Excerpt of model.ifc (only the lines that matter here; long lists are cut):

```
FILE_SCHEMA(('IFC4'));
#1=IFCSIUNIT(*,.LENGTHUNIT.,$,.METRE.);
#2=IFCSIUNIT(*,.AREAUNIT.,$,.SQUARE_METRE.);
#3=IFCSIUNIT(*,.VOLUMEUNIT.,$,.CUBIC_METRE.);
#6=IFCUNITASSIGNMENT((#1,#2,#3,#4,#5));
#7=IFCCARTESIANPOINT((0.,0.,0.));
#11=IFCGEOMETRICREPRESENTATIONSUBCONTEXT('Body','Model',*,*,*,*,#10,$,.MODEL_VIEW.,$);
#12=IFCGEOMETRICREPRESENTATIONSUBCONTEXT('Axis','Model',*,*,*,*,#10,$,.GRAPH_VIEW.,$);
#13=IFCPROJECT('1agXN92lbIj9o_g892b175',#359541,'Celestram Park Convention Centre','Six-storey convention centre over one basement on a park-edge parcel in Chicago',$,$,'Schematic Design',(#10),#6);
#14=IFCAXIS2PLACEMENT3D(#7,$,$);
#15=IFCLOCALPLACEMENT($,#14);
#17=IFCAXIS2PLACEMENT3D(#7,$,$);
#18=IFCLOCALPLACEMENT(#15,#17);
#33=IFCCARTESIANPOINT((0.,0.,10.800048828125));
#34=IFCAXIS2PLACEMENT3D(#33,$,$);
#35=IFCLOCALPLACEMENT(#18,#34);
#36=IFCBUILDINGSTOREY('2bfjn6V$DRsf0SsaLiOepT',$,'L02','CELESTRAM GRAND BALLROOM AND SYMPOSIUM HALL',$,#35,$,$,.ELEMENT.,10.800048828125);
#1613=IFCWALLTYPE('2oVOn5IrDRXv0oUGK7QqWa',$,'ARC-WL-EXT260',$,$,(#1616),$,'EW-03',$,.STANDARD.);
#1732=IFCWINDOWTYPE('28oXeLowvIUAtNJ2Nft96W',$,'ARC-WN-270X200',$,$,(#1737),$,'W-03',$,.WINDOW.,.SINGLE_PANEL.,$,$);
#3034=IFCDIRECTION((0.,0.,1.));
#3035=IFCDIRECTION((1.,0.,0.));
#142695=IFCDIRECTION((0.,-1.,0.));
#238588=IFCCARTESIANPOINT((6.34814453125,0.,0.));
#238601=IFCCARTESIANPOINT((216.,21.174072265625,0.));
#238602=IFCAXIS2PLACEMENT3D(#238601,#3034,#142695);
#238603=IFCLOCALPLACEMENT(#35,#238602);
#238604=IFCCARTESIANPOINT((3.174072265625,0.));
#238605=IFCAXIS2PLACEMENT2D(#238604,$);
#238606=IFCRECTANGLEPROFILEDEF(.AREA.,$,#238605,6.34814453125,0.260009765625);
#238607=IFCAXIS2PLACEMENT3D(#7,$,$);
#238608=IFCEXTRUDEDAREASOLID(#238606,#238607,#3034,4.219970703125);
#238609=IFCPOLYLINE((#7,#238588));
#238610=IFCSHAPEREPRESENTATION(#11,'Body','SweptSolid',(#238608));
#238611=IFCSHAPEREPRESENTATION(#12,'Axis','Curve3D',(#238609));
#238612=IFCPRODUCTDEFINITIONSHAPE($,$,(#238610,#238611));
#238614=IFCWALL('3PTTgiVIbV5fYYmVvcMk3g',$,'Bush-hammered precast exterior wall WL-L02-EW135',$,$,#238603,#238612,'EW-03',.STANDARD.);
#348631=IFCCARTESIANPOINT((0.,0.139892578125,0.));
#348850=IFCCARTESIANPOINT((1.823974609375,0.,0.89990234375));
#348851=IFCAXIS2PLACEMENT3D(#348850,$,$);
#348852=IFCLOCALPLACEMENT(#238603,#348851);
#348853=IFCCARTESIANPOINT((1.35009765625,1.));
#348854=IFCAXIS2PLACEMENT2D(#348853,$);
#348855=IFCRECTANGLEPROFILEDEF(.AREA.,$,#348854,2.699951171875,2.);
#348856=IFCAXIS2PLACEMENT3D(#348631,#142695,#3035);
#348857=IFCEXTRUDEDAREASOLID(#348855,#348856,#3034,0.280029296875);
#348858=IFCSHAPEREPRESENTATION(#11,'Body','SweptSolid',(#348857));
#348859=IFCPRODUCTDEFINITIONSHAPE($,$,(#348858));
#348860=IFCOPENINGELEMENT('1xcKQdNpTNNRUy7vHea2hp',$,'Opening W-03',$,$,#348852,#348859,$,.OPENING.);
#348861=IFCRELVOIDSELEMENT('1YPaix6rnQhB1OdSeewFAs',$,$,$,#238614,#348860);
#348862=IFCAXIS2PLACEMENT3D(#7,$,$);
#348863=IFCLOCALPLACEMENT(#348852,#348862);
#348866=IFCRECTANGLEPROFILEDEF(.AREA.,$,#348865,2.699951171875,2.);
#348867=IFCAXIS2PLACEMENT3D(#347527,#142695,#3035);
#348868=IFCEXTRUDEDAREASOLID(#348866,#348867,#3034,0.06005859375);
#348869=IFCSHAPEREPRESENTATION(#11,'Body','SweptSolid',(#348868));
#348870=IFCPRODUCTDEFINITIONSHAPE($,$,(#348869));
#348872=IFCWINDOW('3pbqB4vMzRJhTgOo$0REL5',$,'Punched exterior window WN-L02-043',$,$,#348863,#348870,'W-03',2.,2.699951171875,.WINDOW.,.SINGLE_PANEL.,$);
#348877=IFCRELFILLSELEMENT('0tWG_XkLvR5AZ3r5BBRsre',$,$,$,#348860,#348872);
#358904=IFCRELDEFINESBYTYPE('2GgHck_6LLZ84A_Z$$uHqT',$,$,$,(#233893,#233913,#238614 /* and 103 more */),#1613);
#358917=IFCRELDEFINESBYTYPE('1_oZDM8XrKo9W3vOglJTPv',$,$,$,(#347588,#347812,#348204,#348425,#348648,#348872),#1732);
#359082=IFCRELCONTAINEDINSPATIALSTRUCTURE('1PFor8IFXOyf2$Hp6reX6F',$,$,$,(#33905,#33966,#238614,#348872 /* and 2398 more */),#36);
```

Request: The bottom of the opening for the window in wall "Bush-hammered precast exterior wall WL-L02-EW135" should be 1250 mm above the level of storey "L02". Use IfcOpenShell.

```python
import numpy as np
import ifcopenshell
import ifcopenshell.api.geometry
import ifcopenshell.geom
import ifcopenshell.util.element
import ifcopenshell.util.placement
import ifcopenshell.util.shape
import ifcopenshell.util.unit

model = ifcopenshell.open("model.ifc")
unit_scale = ifcopenshell.util.unit.calculate_unit_scale(model)

window = model.by_id(348872)
opening = window.FillsVoids[0].RelatingOpeningElement
storey = ifcopenshell.util.element.get_container(window, ifc_class="IfcBuildingStorey")
level = ifcopenshell.util.placement.get_local_placement(storey.ObjectPlacement)[2, 3]

# The opening's origin need not be at the sill, so measure its lowest point.
shape = ifcopenshell.geom.create_shape(ifcopenshell.geom.settings(), opening)
bottom = ifcopenshell.util.shape.get_shape_bottom_elevation(shape, shape.geometry) / unit_scale
dz = level + 1.25 - bottom

shift = np.array([0.0, 0.0, dz])
# The window is placed relative to its opening, so it follows when the opening moves.
matrix = ifcopenshell.util.placement.get_local_placement(opening.ObjectPlacement)
matrix[:3, 3] += shift
ifcopenshell.api.geometry.edit_object_placement(
    model, product=opening, matrix=matrix, is_si=False, should_transform_children=True
)

print(f"moved by {dz * unit_scale:+.3f} m")

model.write("model-out.ifc")
```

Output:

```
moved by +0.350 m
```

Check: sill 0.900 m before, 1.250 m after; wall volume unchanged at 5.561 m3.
